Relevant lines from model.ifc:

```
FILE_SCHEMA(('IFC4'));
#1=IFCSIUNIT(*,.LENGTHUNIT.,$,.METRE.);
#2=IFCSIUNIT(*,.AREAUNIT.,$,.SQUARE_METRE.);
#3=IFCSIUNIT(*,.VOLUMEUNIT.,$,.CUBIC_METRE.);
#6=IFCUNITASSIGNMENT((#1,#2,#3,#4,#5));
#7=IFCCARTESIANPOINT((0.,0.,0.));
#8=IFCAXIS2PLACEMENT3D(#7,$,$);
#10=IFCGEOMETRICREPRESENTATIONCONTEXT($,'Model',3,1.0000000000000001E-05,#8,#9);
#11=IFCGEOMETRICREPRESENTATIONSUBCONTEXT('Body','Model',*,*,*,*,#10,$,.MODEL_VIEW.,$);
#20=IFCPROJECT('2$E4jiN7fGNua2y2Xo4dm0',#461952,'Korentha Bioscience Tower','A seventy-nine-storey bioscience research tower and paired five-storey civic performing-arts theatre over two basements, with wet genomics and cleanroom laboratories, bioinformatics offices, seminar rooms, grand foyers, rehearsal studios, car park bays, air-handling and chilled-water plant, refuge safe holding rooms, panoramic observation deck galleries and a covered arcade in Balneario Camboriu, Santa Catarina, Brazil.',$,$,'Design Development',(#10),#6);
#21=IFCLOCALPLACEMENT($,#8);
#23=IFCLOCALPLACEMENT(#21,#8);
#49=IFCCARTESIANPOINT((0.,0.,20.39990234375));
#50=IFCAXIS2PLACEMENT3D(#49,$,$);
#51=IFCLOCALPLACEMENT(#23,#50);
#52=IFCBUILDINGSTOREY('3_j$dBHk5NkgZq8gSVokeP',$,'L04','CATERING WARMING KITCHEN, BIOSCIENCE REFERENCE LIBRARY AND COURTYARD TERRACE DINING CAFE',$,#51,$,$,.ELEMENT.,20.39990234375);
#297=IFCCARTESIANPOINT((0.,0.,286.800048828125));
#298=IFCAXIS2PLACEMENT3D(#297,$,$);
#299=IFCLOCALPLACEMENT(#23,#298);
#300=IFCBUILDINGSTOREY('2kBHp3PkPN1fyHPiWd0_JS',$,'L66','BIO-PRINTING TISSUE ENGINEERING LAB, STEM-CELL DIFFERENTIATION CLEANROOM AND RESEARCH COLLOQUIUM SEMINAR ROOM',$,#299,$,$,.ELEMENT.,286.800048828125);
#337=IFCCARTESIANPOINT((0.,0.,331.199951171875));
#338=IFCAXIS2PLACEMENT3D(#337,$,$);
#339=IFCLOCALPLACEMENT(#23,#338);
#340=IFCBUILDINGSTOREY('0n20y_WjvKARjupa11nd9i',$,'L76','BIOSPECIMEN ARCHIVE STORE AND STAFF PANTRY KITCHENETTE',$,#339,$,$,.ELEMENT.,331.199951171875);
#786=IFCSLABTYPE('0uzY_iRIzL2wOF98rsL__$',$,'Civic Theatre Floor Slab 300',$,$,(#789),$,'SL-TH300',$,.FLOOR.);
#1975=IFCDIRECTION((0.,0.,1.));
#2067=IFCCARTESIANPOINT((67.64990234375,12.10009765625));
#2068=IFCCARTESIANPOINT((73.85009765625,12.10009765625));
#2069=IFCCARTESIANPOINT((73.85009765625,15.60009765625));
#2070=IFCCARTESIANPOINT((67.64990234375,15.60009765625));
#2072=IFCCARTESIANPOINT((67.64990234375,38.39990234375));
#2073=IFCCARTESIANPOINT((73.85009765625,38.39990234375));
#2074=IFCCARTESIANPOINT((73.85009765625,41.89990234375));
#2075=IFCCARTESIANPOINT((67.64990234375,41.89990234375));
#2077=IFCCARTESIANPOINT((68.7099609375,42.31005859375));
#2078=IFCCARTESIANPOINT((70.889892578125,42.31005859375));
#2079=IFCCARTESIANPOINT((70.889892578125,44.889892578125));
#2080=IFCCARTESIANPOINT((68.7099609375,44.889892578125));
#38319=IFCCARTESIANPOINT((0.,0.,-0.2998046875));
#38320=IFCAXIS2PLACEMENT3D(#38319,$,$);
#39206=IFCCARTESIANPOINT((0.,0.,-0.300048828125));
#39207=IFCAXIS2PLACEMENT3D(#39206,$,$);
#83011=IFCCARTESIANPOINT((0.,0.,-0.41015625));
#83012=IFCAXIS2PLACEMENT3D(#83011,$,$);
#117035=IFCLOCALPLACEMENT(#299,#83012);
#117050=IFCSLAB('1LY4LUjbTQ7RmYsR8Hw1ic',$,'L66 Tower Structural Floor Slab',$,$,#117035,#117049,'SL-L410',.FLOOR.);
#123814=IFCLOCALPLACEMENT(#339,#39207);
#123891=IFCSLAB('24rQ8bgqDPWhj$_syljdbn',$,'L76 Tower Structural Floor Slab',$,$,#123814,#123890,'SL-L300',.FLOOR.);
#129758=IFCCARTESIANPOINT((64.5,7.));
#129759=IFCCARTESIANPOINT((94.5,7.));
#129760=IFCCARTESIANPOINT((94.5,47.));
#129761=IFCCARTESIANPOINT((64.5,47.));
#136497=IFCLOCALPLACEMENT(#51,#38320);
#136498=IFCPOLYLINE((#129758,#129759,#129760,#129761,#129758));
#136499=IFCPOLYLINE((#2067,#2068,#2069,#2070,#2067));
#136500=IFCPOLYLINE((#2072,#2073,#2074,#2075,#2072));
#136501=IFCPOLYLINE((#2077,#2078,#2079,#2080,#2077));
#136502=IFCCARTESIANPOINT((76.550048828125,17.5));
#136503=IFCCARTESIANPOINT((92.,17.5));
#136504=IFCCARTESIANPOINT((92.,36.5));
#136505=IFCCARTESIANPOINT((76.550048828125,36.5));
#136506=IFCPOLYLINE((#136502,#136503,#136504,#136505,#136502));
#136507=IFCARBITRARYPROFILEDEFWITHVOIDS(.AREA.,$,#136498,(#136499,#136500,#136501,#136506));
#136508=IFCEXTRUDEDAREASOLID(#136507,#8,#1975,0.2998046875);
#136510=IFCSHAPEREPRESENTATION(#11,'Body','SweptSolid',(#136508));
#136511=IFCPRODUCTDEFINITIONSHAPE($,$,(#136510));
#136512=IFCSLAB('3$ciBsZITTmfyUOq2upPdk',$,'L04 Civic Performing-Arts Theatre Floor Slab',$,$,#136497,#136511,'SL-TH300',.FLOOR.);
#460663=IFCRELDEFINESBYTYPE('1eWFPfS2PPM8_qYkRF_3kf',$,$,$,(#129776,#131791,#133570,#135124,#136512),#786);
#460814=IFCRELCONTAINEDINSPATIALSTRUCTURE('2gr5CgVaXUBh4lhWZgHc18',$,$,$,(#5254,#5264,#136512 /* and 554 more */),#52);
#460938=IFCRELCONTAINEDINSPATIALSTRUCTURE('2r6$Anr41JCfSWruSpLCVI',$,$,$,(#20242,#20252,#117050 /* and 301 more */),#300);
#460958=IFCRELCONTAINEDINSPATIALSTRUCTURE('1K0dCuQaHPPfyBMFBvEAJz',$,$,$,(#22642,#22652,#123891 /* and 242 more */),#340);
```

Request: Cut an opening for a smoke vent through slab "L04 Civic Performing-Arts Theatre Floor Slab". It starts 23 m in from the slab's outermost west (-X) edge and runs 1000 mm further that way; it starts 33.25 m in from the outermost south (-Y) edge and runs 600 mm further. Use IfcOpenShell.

```python
import numpy as np
import ifcopenshell
import ifcopenshell.api.feature
import ifcopenshell.api.geometry
import ifcopenshell.api.root
import ifcopenshell.geom
import ifcopenshell.util.placement
import ifcopenshell.util.representation
import ifcopenshell.util.shape
import ifcopenshell.util.unit

model = ifcopenshell.open("model.ifc")
unit_scale = ifcopenshell.util.unit.calculate_unit_scale(model)
settings = ifcopenshell.geom.settings()


def volume(element):
    """Net volume in cubic metres, openings subtracted."""
    shape = ifcopenshell.geom.create_shape(settings, element)
    return ifcopenshell.util.shape.get_volume(shape.geometry)


slab = model.by_guid("3$ciBsZITTmfyUOq2upPdk")
before = volume(slab)

# Extent in the slab's own axes, in metres. The edges named are its -X and -Y sides.
slab_shape = ifcopenshell.geom.create_shape(settings, slab)
vertices = ifcopenshell.util.shape.get_vertices(slab_shape.geometry)
x_min, y_min, bottom = vertices.min(axis=0)
top = vertices[:, 2].max()

opening = ifcopenshell.api.root.create_entity(model, ifc_class="IfcOpeningElement", name="Smoke vent opening", predefined_type="OPENING")
context = ifcopenshell.util.representation.get_context(model, "Model", "Body", "MODEL_VIEW")
width, depth = 1, 0.6
outline = [(0.0, 0.0), (width, 0.0), (width, depth), (0.0, depth), (0.0, 0.0)]
# Overshoot both faces by 50 mm so the cut is clean.
shape = ifcopenshell.api.geometry.add_slab_representation(
    model, context=context, depth=top - bottom + 0.1, polyline=outline
)
ifcopenshell.api.geometry.assign_representation(model, product=opening, representation=shape)

matrix = ifcopenshell.util.placement.get_local_placement(slab.ObjectPlacement)
matrix[:, 3] = matrix @ np.append(np.array([x_min + 23, y_min + 33.25, bottom - 0.05]) / unit_scale, 1.0)
ifcopenshell.api.geometry.edit_object_placement(model, product=opening, matrix=matrix, is_si=False)
ifcopenshell.api.feature.add_feature(model, feature=opening, element=slab)

after = volume(slab)

print(f"slab volume {before:.3f} -> {after:.3f} m3")

model.write("model-out.ifc")
```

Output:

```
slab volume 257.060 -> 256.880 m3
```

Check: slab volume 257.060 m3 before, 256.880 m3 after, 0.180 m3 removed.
